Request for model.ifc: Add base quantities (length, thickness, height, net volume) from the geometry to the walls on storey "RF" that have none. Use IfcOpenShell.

First a look at what the model holds.

```python
import ifcopenshell
import ifcopenshell.util.element
import ifcopenshell.util.unit

model = ifcopenshell.open("model.ifc")
print(model.schema)
for unit_type in ("LENGTHUNIT", "AREAUNIT", "VOLUMEUNIT"):
    print(unit_type, ifcopenshell.util.unit.calculate_unit_scale(model, unit_type))
storey = next(s for s in model.by_type("IfcBuildingStorey") if s.Name == "RF")
walls = [e for e in ifcopenshell.util.element.get_decomposition(storey) if e.is_a("IfcWall")]
for e in sorted(walls, key=lambda e: e.id()):
    print(e.id(), e.is_a(), e.Name, list(ifcopenshell.util.element.get_psets(e, qtos_only=True)), sep=" | ")
```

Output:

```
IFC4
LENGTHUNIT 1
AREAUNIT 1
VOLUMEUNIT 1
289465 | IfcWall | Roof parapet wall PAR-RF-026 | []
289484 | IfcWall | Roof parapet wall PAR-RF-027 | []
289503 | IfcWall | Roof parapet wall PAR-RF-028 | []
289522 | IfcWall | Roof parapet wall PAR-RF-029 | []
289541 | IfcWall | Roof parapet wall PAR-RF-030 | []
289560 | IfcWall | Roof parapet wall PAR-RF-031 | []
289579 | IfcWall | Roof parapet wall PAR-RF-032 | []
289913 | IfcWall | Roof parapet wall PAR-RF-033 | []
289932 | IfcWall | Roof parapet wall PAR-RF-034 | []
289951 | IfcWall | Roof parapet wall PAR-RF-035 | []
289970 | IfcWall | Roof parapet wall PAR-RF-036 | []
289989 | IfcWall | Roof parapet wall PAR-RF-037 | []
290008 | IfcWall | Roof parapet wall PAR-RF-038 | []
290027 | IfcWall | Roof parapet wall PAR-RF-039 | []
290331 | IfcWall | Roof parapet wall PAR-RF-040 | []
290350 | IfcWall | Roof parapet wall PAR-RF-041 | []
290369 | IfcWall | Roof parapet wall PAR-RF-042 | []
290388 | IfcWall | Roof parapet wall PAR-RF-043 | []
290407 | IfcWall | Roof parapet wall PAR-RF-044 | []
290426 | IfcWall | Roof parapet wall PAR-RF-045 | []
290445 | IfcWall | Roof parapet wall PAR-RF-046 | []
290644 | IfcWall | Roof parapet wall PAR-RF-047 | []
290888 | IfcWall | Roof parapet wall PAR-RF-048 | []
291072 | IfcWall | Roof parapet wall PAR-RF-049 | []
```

```python
import ifcopenshell
import ifcopenshell.api.pset
import ifcopenshell.geom
import ifcopenshell.util.element
import ifcopenshell.util.shape
import ifcopenshell.util.unit

model = ifcopenshell.open("model.ifc")
unit_scale = ifcopenshell.util.unit.calculate_unit_scale(model)
volume_scale = ifcopenshell.util.unit.calculate_unit_scale(model, "VOLUMEUNIT")
settings = ifcopenshell.geom.settings()

storey = next(s for s in model.by_type("IfcBuildingStorey") if s.Name == "RF")
walls = [e for e in ifcopenshell.util.element.get_decomposition(storey) if e.is_a("IfcWall")]

for e in sorted(walls, key=lambda e: e.id()):
    if ifcopenshell.util.element.get_psets(e, qtos_only=True, should_inherit=False):
        continue
    # Geometry comes back in metres, in the element's own axes.
    shape = ifcopenshell.geom.create_shape(settings, e)
    values = {
        "Length": ifcopenshell.util.shape.get_x(shape.geometry) / unit_scale,
        "Width": ifcopenshell.util.shape.get_y(shape.geometry) / unit_scale,
        "Height": ifcopenshell.util.shape.get_z(shape.geometry) / unit_scale,
        "NetVolume": ifcopenshell.util.shape.get_volume(shape.geometry) / volume_scale,
    }
    qto = ifcopenshell.api.pset.add_qto(model, product=e, name="Qto_WallBaseQuantities")
    ifcopenshell.api.pset.edit_qto(model, qto=qto, properties=values)
    print(e.id(), {k: round(v, 3) for k, v in values.items()})

model.write("model-out.ifc")
```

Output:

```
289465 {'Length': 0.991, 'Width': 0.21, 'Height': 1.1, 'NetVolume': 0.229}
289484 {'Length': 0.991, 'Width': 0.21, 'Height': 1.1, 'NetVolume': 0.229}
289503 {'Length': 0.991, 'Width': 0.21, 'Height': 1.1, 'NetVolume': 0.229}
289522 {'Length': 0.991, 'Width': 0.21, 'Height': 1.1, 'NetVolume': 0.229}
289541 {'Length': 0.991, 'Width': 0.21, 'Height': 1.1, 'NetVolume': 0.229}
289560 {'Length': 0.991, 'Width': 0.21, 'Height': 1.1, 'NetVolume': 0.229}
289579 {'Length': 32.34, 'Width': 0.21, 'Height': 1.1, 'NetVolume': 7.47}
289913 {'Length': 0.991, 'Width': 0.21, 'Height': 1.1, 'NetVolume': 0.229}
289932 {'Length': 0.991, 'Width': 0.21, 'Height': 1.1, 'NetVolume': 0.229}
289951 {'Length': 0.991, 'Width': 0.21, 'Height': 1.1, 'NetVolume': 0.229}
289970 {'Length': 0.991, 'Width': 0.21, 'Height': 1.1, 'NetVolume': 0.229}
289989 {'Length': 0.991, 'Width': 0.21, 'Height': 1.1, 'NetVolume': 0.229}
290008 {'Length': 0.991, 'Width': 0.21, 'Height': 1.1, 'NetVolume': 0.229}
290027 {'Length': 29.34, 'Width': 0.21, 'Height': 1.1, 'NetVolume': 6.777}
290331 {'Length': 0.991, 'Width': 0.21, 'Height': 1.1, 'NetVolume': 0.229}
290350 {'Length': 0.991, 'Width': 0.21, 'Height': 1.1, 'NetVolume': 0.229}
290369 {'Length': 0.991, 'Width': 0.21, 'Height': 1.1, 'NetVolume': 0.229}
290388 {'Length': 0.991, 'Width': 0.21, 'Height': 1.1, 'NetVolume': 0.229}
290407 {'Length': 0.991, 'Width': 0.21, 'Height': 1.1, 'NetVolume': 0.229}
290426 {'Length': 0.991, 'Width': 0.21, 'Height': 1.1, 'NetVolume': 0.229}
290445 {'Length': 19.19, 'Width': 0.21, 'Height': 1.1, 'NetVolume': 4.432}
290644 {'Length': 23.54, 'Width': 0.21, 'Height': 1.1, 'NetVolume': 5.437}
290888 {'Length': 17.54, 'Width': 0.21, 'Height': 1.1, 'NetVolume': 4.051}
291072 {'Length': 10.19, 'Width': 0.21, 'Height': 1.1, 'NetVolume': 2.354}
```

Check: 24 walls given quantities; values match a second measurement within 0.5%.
